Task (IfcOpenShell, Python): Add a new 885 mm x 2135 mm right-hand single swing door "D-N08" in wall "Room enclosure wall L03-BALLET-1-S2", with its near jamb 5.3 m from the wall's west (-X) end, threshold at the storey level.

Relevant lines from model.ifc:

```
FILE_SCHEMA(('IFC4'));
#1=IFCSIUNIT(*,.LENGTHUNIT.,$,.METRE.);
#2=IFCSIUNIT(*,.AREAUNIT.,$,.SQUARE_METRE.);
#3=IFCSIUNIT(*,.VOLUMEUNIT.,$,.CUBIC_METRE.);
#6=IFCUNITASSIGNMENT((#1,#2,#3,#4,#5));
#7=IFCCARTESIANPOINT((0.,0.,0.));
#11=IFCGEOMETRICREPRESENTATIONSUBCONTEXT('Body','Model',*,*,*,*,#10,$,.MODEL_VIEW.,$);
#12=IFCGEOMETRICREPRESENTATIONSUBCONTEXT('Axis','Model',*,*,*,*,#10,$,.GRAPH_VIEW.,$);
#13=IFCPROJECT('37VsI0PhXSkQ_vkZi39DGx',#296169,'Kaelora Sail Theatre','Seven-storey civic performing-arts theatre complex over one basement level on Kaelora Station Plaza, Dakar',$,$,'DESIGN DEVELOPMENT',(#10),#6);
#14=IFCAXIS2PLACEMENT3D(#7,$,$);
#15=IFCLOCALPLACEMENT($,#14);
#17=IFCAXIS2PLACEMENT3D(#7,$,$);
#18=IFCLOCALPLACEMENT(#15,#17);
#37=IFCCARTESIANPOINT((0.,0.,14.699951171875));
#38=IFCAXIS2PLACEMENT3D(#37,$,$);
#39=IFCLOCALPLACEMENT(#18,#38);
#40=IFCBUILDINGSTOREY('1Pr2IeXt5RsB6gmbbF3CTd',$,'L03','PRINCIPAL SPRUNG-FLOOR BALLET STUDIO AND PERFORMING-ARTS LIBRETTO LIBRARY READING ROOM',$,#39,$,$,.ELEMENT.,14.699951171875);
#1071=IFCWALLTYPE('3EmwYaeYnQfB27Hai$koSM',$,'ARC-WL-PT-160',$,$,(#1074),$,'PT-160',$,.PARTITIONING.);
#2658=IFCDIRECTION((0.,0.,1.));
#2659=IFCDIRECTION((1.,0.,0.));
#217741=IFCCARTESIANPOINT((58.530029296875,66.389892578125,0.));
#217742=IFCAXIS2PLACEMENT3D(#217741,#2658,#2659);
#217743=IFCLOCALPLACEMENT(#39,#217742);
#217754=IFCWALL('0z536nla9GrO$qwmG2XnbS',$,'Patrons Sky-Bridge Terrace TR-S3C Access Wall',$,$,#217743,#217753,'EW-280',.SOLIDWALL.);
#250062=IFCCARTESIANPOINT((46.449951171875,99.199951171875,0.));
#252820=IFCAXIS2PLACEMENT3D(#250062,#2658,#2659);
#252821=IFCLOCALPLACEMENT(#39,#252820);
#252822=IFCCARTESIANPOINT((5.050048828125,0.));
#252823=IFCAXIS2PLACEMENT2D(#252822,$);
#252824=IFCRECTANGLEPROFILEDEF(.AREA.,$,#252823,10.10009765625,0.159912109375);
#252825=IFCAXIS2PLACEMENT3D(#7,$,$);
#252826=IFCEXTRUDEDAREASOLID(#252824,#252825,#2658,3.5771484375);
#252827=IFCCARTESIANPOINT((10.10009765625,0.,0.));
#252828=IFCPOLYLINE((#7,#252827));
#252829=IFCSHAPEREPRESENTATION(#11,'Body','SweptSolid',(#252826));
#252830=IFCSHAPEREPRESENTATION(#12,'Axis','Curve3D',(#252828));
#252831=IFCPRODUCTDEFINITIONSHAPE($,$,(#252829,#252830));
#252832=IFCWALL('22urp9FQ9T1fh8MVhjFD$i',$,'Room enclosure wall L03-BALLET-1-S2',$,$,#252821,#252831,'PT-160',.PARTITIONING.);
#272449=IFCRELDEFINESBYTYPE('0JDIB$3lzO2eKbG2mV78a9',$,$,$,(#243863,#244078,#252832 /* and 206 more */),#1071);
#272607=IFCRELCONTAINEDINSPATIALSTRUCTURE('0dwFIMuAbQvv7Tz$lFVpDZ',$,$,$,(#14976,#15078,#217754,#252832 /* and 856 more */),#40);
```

```python
import numpy as np
import ifcopenshell
import ifcopenshell.api.feature
import ifcopenshell.api.geometry
import ifcopenshell.api.root
import ifcopenshell.api.spatial
import ifcopenshell.geom
import ifcopenshell.util.element
import ifcopenshell.util.placement
import ifcopenshell.util.representation
import ifcopenshell.util.shape
import ifcopenshell.util.unit

model = ifcopenshell.open("model.ifc")
unit_scale = ifcopenshell.util.unit.calculate_unit_scale(model)
settings = ifcopenshell.geom.settings()


def volume(element):
    """Net volume in cubic metres, openings subtracted."""
    shape = ifcopenshell.geom.create_shape(settings, element)
    return ifcopenshell.util.shape.get_volume(shape.geometry)


wall = model.by_id(252832)
storey = ifcopenshell.util.element.get_container(wall, ifc_class="IfcBuildingStorey")
context = ifcopenshell.util.representation.get_context(model, "Model", "Body", "MODEL_VIEW")
before = volume(wall)

width, height, from_end, sill = 0.885, 2.135, 5.3, 0.0  # metres

# The wall runs along its own X axis, and the end named is its -X end.
wall_shape = ifcopenshell.geom.create_shape(settings, wall)
x, y, z = ifcopenshell.util.shape.get_vertices(wall_shape.geometry).T
start = x.min() + from_end
face, thickness = float(y.min()), float(y.max() - y.min())
wall_matrix = ifcopenshell.util.placement.get_local_placement(wall.ObjectPlacement)
level = ifcopenshell.util.placement.get_local_placement(storey.ObjectPlacement)[2, 3]


def in_wall(x, y):
    """Placement at x, y metres in the wall's axes, at sill height."""
    matrix = wall_matrix.copy()
    matrix[:, 3] = wall_matrix @ np.array([x / unit_scale, y / unit_scale, 0.0, 1.0])
    matrix[2, 3] = level + sill / unit_scale
    return matrix


# Opening: a box that overshoots both wall faces by 50 mm.
opening = ifcopenshell.api.root.create_entity(model, ifc_class="IfcOpeningElement", predefined_type="OPENING")
box = ifcopenshell.api.geometry.add_wall_representation(
    model, context=context, length=width, height=height, thickness=thickness + 0.1
)
ifcopenshell.api.geometry.assign_representation(model, product=opening, representation=box)
ifcopenshell.api.geometry.edit_object_placement(model, product=opening, matrix=in_wall(start, face - 0.05), is_si=False)
ifcopenshell.api.feature.add_feature(model, feature=opening, element=wall)

door = ifcopenshell.api.root.create_entity(model, ifc_class="IfcDoor", name="D-N08", predefined_type="DOOR")
door.OverallWidth, door.OverallHeight = width / unit_scale, height / unit_scale
door.OperationType = "SINGLE_SWING_RIGHT"
body = ifcopenshell.api.geometry.add_door_representation(
    model,
    context=context,
    overall_width=door.OverallWidth,
    overall_height=door.OverallHeight,
    operation_type="SINGLE_SWING_RIGHT",
    lining_properties={"LiningDepth": thickness / unit_scale, "ThresholdDepth": thickness / unit_scale},
)
ifcopenshell.api.geometry.assign_representation(model, product=door, representation=body)
ifcopenshell.api.spatial.assign_container(model, products=[door], relating_structure=storey)
ifcopenshell.api.feature.add_filling(model, opening=opening, element=door)

# The lining spans the wall, so the door starts at the wall face.
ifcopenshell.api.geometry.edit_object_placement(model, product=door, matrix=in_wall(start, face), is_si=False)

after = volume(wall)

print(f"wall volume {before:.3f} -> {after:.3f} m3")

model.write("model_v2.ifc")
```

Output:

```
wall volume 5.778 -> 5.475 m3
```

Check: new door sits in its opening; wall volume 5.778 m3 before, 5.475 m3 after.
